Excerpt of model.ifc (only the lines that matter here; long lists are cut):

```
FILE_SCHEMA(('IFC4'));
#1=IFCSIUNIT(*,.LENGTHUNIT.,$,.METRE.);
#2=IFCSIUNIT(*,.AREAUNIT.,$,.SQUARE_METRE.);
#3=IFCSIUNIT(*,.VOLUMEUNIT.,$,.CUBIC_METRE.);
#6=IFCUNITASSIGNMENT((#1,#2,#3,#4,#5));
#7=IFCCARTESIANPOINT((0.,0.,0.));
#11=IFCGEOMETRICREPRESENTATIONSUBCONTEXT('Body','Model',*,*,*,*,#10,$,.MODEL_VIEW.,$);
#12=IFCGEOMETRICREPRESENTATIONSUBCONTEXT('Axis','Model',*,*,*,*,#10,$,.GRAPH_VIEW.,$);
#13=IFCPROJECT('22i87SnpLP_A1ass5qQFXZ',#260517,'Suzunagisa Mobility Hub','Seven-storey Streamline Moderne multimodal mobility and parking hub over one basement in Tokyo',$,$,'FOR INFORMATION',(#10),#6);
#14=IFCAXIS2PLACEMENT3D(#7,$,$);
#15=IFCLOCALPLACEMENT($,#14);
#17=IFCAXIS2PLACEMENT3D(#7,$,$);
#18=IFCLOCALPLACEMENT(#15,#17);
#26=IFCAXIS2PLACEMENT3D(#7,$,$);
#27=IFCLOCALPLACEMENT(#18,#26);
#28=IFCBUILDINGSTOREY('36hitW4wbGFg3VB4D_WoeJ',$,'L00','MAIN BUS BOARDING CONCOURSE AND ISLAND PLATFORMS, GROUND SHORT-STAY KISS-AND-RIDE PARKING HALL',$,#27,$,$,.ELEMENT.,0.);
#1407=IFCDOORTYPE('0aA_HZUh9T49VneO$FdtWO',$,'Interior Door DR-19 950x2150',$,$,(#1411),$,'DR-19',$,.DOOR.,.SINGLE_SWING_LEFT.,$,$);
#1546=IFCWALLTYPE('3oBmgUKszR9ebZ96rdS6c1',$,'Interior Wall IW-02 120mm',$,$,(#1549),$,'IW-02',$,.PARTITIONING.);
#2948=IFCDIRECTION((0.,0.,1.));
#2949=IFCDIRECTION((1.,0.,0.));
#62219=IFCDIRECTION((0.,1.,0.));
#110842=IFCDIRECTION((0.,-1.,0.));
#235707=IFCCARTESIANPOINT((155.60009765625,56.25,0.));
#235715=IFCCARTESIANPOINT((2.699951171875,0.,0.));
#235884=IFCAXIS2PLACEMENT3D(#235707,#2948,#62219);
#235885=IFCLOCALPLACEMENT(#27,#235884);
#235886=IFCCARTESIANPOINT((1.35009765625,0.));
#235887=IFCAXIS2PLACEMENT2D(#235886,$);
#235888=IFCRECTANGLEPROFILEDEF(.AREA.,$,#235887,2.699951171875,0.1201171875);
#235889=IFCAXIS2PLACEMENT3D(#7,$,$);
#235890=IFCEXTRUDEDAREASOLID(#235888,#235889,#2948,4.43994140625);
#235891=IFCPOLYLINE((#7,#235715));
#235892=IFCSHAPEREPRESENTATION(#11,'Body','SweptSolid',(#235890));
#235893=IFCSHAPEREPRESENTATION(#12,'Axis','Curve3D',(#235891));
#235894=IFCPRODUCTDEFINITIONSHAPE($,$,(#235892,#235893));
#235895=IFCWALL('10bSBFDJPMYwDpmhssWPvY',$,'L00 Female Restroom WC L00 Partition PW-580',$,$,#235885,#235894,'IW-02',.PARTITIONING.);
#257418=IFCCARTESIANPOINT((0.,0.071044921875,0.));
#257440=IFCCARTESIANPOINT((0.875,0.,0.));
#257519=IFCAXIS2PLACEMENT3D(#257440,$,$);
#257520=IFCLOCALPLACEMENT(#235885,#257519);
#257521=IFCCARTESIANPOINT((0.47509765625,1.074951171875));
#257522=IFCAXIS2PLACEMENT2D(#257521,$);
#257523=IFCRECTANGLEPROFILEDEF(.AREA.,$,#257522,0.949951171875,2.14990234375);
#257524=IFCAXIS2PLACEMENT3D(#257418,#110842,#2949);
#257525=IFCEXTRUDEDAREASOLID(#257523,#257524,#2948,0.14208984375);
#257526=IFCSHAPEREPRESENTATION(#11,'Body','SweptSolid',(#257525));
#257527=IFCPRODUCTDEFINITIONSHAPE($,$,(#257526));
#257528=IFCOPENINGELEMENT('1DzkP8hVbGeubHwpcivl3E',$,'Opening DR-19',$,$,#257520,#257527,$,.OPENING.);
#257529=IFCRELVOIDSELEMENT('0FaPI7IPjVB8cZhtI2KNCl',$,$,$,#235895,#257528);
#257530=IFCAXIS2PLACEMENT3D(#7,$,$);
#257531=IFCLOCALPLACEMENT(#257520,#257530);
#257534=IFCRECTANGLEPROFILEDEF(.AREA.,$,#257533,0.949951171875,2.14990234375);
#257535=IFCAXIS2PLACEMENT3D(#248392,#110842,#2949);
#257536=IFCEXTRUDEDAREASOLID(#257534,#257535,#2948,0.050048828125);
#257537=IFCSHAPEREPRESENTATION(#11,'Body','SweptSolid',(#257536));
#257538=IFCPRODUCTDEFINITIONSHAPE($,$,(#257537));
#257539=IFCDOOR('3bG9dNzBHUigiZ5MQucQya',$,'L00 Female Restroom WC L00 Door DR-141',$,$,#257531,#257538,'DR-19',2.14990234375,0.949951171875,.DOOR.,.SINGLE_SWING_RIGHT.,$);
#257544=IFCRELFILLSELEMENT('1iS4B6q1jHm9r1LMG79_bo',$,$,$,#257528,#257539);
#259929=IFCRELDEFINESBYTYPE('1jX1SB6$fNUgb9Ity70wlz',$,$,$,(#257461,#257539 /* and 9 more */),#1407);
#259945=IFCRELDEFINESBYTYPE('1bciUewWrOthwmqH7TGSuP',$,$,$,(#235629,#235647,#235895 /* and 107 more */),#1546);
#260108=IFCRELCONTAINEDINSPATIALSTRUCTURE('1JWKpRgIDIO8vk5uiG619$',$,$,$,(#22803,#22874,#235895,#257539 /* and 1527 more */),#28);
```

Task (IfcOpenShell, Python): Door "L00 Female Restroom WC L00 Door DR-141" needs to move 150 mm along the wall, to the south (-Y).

```python
import ifcopenshell
import ifcopenshell.api.geometry
import ifcopenshell.util.placement
import ifcopenshell.util.unit

model = ifcopenshell.open("model.ifc")
unit_scale = ifcopenshell.util.unit.calculate_unit_scale(model)

door = model.by_guid("3bG9dNzBHUigiZ5MQucQya")
opening = door.FillsVoids[0].RelatingOpeningElement
wall = opening.VoidsElements[0].RelatingBuildingElement

wall_matrix = ifcopenshell.util.placement.get_local_placement(wall.ObjectPlacement)
shift = wall_matrix[:3, 0] * -0.15 / unit_scale
before = ifcopenshell.util.placement.get_local_placement(door.ObjectPlacement)[:3, 3].copy()

# The door is placed relative to its opening, so it follows when the opening moves.
matrix = ifcopenshell.util.placement.get_local_placement(opening.ObjectPlacement)
matrix[:3, 3] += shift
ifcopenshell.api.geometry.edit_object_placement(
    model, product=opening, matrix=matrix, is_si=False, should_transform_children=True
)

after = ifcopenshell.util.placement.get_local_placement(door.ObjectPlacement)[:3, 3]
print("door moved by", (after - before).round(3) + 0.0)

model.write("model_rev.ifc")
```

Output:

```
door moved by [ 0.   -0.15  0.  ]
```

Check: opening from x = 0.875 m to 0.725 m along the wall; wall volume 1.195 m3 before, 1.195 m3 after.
